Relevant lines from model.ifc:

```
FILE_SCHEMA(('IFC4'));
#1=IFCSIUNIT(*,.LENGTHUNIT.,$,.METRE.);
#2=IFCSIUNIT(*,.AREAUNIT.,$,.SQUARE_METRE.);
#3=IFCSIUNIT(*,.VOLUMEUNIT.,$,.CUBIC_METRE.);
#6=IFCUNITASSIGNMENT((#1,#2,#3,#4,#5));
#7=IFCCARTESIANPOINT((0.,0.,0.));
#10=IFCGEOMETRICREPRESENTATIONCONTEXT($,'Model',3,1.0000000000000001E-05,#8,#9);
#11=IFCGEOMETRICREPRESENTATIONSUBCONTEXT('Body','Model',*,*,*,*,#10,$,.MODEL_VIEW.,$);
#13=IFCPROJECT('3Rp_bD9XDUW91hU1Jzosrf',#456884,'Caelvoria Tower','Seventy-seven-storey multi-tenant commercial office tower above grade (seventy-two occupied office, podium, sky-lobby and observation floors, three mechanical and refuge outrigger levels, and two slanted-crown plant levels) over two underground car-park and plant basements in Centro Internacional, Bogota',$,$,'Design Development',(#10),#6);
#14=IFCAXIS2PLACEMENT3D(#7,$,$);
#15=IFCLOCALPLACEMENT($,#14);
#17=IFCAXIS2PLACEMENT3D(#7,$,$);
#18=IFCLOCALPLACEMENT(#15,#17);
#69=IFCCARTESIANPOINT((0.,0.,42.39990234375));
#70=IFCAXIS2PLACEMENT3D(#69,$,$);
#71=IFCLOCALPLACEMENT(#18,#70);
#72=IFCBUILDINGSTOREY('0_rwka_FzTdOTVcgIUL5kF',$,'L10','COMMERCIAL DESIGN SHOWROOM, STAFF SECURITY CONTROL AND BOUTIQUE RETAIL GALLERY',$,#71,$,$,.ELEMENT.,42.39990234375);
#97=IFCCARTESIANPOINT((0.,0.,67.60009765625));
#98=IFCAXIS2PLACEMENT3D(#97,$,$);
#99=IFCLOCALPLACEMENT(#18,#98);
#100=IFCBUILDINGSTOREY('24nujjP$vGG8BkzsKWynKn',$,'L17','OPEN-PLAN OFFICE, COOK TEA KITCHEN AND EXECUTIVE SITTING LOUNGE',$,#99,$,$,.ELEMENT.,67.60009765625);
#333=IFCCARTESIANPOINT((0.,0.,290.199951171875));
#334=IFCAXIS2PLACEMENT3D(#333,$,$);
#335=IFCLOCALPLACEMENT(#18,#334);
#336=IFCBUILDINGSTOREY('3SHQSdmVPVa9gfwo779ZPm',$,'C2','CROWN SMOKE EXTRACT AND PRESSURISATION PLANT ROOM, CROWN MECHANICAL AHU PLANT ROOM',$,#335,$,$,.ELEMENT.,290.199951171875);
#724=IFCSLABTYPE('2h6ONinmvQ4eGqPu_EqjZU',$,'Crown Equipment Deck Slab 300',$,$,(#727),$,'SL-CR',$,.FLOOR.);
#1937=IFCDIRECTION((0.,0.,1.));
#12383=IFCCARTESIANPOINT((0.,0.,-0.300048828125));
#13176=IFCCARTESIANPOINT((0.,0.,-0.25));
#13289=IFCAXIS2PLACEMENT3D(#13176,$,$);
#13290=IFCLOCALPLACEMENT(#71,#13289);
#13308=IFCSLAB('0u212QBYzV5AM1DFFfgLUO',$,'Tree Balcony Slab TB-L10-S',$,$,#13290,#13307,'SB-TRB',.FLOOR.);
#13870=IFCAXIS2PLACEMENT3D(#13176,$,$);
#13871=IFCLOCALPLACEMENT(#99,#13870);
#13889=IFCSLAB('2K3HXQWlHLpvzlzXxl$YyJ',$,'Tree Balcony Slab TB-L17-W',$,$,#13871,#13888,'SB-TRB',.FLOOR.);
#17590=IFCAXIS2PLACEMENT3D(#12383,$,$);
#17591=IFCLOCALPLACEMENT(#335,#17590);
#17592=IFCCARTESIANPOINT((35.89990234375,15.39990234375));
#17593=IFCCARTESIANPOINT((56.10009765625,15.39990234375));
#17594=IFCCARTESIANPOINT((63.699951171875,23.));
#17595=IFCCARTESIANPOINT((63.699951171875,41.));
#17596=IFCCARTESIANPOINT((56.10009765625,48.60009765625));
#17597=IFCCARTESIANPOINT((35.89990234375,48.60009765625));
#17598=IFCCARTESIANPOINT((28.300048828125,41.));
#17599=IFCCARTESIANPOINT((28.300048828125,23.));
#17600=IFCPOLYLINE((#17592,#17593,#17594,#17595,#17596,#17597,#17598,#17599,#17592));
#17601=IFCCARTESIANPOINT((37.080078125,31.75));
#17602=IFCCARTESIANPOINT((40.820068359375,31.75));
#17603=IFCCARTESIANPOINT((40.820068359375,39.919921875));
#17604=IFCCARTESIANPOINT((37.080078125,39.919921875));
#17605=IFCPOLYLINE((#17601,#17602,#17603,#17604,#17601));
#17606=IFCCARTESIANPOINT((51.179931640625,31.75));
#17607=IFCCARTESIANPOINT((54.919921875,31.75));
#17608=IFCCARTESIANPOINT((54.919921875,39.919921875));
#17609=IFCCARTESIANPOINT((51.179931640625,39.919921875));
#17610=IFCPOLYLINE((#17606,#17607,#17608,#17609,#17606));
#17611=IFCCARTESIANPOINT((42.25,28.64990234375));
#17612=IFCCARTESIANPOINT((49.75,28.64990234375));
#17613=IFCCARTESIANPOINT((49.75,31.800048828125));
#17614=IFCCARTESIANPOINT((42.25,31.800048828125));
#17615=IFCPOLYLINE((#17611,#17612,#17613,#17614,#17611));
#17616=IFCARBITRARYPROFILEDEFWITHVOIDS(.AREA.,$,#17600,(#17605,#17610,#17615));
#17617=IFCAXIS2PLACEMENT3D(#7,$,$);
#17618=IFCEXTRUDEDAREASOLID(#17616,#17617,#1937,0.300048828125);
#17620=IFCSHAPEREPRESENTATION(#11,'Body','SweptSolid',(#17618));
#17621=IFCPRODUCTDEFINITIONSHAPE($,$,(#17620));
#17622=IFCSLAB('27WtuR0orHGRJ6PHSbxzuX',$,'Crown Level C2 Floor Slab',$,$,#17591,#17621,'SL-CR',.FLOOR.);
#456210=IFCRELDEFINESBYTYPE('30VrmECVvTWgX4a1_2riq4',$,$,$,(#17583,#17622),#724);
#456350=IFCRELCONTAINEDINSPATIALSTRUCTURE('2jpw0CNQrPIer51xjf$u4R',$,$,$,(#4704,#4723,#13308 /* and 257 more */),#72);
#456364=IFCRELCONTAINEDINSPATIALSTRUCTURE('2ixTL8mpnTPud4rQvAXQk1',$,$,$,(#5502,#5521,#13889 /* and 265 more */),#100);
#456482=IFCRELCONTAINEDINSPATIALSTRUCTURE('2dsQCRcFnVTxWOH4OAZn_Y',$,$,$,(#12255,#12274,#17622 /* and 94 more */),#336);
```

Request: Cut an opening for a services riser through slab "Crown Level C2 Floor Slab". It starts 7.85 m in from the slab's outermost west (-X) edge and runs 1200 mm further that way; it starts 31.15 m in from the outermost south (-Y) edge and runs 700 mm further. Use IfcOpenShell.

```python
import numpy as np
import ifcopenshell
import ifcopenshell.api.feature
import ifcopenshell.api.geometry
import ifcopenshell.api.root
import ifcopenshell.geom
import ifcopenshell.util.placement
import ifcopenshell.util.representation
import ifcopenshell.util.shape
import ifcopenshell.util.unit

model = ifcopenshell.open("model.ifc")
unit_scale = ifcopenshell.util.unit.calculate_unit_scale(model)
settings = ifcopenshell.geom.settings()


def volume(element):
    """Net volume in cubic metres, openings subtracted."""
    shape = ifcopenshell.geom.create_shape(settings, element)
    return ifcopenshell.util.shape.get_volume(shape.geometry)


slab = model.by_guid("27WtuR0orHGRJ6PHSbxzuX")
before = volume(slab)

# Extent in the slab's own axes, in metres. The edges named are its -X and -Y sides.
slab_shape = ifcopenshell.geom.create_shape(settings, slab)
vertices = ifcopenshell.util.shape.get_vertices(slab_shape.geometry)
x_min, y_min, bottom = vertices.min(axis=0)
top = vertices[:, 2].max()

opening = ifcopenshell.api.root.create_entity(model, ifc_class="IfcOpeningElement", name="Services riser opening", predefined_type="OPENING")
context = ifcopenshell.util.representation.get_context(model, "Model", "Body", "MODEL_VIEW")
width, depth = 1.2, 0.7
outline = [(0.0, 0.0), (width, 0.0), (width, depth), (0.0, depth), (0.0, 0.0)]
# Overshoot both faces by 50 mm so the cut is clean.
shape = ifcopenshell.api.geometry.add_slab_representation(
    model, context=context, depth=top - bottom + 0.1, polyline=outline
)
ifcopenshell.api.geometry.assign_representation(model, product=opening, representation=shape)

matrix = ifcopenshell.util.placement.get_local_placement(slab.ObjectPlacement)
matrix[:, 3] = matrix @ np.append(np.array([x_min + 7.85, y_min + 31.15, bottom - 0.05]) / unit_scale, 1.0)
ifcopenshell.api.geometry.edit_object_placement(model, product=opening, matrix=matrix, is_si=False)
ifcopenshell.api.feature.add_feature(model, feature=opening, element=slab)

after = volume(slab)

print(f"slab volume {before:.3f} -> {after:.3f} m3")

model.write("model_edited.ifc")
```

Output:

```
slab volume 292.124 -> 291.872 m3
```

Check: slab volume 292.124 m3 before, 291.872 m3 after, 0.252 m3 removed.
